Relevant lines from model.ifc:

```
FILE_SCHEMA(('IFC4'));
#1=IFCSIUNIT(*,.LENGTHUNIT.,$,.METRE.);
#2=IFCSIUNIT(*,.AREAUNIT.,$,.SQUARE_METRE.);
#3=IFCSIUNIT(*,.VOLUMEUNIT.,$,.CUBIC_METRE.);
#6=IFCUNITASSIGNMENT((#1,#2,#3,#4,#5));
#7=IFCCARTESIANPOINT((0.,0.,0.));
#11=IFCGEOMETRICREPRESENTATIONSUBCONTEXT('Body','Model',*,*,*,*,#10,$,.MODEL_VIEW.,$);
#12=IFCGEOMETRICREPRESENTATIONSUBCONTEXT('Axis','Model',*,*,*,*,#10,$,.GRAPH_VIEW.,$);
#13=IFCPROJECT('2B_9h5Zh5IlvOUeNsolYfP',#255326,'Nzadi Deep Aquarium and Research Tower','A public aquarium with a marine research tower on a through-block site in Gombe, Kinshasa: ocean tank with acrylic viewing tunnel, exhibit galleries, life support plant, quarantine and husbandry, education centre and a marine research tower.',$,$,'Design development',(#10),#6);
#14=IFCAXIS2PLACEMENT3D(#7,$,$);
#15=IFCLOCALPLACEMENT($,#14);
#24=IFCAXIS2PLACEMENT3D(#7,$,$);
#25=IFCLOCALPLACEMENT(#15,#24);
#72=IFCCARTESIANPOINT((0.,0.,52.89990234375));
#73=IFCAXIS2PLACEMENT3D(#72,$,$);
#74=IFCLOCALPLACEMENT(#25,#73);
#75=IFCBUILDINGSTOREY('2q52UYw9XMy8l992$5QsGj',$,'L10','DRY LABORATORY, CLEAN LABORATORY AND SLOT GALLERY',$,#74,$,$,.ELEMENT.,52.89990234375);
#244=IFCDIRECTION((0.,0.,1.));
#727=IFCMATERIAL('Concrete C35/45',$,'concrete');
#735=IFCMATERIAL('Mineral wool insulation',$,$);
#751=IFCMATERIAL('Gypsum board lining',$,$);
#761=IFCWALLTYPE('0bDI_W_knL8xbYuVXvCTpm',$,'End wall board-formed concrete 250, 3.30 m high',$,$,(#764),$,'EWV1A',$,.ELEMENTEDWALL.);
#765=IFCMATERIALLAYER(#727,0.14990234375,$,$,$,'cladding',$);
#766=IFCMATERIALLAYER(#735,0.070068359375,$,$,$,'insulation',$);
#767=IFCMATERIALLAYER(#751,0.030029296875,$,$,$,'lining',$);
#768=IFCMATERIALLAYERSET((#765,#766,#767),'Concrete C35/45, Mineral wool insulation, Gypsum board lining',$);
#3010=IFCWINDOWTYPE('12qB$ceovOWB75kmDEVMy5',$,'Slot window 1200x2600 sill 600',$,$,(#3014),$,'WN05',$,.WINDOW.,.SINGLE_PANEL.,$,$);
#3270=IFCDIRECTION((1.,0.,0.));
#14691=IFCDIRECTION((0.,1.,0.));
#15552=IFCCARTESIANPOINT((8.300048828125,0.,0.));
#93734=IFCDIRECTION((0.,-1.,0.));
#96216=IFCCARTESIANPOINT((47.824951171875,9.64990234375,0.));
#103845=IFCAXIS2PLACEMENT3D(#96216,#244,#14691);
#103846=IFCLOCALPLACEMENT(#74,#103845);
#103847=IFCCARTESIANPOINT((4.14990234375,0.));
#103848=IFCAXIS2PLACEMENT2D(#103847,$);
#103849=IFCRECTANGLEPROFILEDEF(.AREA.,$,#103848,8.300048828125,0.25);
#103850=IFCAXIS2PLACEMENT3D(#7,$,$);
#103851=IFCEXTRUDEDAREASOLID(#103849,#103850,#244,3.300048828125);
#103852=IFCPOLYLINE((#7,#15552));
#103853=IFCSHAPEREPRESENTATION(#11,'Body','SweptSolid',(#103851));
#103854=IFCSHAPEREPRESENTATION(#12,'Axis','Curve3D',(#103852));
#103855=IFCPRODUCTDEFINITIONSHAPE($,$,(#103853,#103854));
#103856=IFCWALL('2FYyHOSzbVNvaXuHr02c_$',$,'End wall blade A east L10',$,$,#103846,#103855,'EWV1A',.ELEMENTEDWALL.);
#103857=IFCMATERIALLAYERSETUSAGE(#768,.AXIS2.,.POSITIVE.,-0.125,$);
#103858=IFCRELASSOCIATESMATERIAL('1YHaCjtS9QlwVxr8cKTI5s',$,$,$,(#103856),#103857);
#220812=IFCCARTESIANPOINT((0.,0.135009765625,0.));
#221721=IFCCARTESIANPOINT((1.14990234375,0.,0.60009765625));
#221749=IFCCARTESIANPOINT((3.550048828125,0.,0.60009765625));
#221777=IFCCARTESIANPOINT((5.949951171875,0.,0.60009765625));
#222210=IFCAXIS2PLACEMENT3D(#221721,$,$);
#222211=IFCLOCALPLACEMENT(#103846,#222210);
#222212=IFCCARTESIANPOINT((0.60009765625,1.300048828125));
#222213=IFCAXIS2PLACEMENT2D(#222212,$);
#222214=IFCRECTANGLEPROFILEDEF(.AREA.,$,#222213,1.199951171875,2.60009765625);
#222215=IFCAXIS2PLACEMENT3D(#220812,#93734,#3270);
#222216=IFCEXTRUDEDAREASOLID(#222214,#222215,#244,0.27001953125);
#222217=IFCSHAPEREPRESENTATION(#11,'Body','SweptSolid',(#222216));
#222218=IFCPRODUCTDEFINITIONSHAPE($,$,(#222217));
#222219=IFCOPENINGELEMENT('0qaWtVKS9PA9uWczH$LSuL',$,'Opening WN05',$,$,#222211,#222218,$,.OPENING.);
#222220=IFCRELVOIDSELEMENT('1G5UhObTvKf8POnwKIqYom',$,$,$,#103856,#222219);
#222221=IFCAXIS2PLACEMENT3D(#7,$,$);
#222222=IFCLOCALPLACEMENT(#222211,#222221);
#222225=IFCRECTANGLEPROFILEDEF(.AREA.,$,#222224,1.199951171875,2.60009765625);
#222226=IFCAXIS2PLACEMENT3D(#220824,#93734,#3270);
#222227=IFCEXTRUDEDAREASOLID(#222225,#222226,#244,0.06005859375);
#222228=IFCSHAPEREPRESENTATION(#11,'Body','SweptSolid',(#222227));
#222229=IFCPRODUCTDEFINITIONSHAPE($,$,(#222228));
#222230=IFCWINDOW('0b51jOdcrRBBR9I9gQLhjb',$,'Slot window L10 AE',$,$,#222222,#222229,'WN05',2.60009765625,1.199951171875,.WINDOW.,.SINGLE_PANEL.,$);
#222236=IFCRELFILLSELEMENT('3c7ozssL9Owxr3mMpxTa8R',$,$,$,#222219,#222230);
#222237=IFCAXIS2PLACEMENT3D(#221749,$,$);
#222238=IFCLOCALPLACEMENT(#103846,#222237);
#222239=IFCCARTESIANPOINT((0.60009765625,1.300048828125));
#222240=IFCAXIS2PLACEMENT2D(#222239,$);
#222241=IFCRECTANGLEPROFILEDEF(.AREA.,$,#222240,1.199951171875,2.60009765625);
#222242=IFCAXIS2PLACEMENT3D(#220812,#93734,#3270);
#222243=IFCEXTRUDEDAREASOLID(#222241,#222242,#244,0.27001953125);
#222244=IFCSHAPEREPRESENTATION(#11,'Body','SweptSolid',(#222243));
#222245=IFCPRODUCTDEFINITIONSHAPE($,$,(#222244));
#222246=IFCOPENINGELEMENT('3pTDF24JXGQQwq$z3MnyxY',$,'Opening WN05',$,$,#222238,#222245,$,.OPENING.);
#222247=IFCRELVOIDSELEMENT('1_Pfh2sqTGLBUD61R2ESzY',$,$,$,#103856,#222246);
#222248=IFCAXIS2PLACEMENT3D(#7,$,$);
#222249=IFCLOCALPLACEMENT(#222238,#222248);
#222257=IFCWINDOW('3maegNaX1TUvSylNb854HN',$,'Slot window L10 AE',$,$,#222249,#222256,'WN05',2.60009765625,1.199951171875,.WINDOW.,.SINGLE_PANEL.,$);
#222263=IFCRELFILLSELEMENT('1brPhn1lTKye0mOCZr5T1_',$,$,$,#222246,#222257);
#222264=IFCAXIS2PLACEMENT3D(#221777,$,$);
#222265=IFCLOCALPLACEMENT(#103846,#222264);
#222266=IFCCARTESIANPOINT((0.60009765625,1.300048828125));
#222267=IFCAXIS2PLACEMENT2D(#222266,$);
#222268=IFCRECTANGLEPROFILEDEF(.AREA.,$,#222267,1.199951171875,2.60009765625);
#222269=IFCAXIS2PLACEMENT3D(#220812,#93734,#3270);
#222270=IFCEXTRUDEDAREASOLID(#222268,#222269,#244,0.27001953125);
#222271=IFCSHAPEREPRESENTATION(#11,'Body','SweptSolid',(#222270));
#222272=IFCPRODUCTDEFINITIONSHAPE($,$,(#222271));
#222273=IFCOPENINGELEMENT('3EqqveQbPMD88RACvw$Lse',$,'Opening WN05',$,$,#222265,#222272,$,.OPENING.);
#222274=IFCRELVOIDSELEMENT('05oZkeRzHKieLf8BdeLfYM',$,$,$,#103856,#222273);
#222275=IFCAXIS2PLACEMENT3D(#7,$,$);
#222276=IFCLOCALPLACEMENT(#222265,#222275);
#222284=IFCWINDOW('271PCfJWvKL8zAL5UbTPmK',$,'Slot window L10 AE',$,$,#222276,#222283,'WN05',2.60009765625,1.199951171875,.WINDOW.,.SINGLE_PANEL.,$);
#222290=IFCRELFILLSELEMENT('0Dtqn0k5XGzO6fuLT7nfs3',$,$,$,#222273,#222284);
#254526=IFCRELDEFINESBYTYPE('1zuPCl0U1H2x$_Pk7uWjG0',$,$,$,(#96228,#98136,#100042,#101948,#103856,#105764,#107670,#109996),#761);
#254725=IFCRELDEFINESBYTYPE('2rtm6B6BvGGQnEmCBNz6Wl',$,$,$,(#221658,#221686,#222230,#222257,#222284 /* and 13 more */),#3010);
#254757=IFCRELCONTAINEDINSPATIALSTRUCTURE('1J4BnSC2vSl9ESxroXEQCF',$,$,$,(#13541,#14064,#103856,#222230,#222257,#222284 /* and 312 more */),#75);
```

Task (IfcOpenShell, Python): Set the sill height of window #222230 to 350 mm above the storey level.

```python
import numpy as np
import ifcopenshell
import ifcopenshell.api.geometry
import ifcopenshell.geom
import ifcopenshell.util.element
import ifcopenshell.util.placement
import ifcopenshell.util.shape
import ifcopenshell.util.unit

model = ifcopenshell.open("model.ifc")
unit_scale = ifcopenshell.util.unit.calculate_unit_scale(model)

window = model.by_guid("0b51jOdcrRBBR9I9gQLhjb")
opening = window.FillsVoids[0].RelatingOpeningElement
storey = ifcopenshell.util.element.get_container(window, ifc_class="IfcBuildingStorey")
level = ifcopenshell.util.placement.get_local_placement(storey.ObjectPlacement)[2, 3]

# The opening's origin need not be at the sill, so measure its lowest point.
shape = ifcopenshell.geom.create_shape(ifcopenshell.geom.settings(), opening)
bottom = ifcopenshell.util.shape.get_shape_bottom_elevation(shape, shape.geometry) / unit_scale
dz = level + 0.35 / unit_scale - bottom

shift = np.array([0.0, 0.0, dz])
# The window is placed relative to its opening, so it follows when the opening moves.
matrix = ifcopenshell.util.placement.get_local_placement(opening.ObjectPlacement)
matrix[:3, 3] += shift
ifcopenshell.api.geometry.edit_object_placement(
    model, product=opening, matrix=matrix, is_si=False, should_transform_children=True
)

print(f"moved by {dz * unit_scale:+.3f} m")

model.write("model_rev.ifc")
```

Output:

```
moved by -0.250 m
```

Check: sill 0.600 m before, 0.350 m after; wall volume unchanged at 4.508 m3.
